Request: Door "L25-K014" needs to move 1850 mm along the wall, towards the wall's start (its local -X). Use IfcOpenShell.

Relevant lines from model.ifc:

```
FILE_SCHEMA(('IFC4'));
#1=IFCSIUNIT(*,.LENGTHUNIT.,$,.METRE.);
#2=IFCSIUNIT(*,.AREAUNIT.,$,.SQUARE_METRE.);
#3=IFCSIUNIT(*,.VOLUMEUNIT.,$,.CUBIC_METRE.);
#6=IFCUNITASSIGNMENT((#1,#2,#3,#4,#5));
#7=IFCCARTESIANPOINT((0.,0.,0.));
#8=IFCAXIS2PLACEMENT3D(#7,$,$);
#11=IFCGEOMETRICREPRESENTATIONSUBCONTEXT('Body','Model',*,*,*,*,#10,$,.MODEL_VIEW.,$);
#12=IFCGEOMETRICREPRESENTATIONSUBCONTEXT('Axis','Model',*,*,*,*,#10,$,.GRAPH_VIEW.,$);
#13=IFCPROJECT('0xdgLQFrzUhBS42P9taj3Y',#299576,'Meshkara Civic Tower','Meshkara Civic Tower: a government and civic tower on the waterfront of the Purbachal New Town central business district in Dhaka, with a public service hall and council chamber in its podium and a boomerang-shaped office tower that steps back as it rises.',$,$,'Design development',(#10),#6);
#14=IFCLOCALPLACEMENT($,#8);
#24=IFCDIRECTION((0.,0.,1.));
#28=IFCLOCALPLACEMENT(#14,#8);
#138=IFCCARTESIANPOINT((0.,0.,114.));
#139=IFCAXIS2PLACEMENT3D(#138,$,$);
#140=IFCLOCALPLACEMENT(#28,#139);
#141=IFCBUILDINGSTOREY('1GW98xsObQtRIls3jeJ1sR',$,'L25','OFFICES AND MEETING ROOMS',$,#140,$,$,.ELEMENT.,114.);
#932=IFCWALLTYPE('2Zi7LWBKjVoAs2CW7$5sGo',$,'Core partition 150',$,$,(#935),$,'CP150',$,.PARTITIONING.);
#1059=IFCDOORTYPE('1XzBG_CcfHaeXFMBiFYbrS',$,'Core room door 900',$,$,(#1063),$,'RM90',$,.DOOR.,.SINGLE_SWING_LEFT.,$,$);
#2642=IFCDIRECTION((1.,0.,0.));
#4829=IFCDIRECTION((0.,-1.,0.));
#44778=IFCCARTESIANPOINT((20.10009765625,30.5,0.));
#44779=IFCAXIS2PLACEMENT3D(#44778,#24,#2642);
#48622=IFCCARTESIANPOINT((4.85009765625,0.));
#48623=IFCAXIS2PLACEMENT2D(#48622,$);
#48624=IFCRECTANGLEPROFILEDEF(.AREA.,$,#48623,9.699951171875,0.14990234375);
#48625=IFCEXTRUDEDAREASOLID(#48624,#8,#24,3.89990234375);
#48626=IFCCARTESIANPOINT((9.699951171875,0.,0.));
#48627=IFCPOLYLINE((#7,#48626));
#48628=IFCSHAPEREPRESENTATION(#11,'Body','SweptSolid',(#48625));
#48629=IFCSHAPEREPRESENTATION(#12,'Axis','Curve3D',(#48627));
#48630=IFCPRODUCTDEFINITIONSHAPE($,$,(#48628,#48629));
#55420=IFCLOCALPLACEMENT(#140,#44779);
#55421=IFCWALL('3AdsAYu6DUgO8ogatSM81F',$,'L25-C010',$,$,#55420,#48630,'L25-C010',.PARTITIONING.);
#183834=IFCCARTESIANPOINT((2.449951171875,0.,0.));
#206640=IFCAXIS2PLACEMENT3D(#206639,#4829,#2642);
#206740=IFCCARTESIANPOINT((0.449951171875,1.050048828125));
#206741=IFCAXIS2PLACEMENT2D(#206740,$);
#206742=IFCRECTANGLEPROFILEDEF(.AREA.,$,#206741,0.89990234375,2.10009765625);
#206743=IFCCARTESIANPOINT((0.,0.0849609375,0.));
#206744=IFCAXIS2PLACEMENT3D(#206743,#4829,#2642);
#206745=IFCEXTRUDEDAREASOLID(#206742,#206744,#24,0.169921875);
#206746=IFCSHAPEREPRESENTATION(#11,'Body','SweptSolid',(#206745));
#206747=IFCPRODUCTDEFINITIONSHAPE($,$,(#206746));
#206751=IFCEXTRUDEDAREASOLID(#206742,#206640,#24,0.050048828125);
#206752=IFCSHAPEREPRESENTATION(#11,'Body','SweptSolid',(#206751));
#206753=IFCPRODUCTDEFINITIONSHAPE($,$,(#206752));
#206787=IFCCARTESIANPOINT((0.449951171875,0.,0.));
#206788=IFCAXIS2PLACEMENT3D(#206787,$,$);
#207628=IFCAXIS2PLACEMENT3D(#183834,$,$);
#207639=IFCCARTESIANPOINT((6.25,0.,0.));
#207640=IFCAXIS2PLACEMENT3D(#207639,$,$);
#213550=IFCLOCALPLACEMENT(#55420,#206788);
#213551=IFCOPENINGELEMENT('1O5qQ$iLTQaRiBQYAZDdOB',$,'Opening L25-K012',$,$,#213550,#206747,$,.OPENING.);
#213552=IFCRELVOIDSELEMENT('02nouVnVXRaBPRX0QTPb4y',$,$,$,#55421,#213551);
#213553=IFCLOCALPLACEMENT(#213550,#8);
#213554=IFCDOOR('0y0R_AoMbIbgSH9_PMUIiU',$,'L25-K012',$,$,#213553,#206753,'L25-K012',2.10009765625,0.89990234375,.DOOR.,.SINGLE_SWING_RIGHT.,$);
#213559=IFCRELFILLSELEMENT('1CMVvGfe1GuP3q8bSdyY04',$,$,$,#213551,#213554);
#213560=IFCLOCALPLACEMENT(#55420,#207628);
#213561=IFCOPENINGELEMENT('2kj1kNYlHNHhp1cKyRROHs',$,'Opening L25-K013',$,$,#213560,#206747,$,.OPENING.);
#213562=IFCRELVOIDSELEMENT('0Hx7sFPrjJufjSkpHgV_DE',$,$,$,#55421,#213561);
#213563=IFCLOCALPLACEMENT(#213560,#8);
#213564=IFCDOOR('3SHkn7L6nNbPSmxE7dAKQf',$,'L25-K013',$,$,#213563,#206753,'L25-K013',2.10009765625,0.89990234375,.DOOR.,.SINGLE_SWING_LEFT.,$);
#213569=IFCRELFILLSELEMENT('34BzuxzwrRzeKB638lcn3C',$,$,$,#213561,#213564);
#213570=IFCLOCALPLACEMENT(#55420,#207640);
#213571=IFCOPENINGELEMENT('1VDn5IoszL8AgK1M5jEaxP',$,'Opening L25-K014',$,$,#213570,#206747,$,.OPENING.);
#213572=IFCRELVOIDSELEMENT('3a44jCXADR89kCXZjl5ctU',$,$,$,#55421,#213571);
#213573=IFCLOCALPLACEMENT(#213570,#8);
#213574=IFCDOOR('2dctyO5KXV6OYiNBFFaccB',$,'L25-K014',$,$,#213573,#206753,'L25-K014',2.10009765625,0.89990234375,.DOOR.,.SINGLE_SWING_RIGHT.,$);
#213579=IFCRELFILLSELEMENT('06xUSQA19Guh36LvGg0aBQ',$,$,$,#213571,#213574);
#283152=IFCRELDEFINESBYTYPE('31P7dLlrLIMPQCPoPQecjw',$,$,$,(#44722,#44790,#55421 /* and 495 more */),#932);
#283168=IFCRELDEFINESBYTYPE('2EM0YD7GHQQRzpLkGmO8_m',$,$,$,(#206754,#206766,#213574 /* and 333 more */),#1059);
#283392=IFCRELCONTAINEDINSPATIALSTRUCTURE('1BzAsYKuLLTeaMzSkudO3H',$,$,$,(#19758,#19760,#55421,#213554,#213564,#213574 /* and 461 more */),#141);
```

```python
import ifcopenshell
import ifcopenshell.api.geometry
import ifcopenshell.util.placement
import ifcopenshell.util.unit

model = ifcopenshell.open("model.ifc")
unit_scale = ifcopenshell.util.unit.calculate_unit_scale(model)

door = model.by_guid("2dctyO5KXV6OYiNBFFaccB")
opening = door.FillsVoids[0].RelatingOpeningElement
wall = opening.VoidsElements[0].RelatingBuildingElement

wall_matrix = ifcopenshell.util.placement.get_local_placement(wall.ObjectPlacement)
shift = wall_matrix[:3, 0] * -1.85 / unit_scale
before = ifcopenshell.util.placement.get_local_placement(door.ObjectPlacement)[:3, 3].copy()

# The door is placed relative to its opening, so it follows when the opening moves.
matrix = ifcopenshell.util.placement.get_local_placement(opening.ObjectPlacement)
matrix[:3, 3] += shift
ifcopenshell.api.geometry.edit_object_placement(
    model, product=opening, matrix=matrix, is_si=False, should_transform_children=True
)

after = ifcopenshell.util.placement.get_local_placement(door.ObjectPlacement)[:3, 3]
print("door moved by", (after - before).round(3) + 0.0)

model.write("model_v2.ifc")
```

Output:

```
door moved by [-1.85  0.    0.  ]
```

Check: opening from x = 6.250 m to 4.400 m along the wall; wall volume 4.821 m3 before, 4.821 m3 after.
